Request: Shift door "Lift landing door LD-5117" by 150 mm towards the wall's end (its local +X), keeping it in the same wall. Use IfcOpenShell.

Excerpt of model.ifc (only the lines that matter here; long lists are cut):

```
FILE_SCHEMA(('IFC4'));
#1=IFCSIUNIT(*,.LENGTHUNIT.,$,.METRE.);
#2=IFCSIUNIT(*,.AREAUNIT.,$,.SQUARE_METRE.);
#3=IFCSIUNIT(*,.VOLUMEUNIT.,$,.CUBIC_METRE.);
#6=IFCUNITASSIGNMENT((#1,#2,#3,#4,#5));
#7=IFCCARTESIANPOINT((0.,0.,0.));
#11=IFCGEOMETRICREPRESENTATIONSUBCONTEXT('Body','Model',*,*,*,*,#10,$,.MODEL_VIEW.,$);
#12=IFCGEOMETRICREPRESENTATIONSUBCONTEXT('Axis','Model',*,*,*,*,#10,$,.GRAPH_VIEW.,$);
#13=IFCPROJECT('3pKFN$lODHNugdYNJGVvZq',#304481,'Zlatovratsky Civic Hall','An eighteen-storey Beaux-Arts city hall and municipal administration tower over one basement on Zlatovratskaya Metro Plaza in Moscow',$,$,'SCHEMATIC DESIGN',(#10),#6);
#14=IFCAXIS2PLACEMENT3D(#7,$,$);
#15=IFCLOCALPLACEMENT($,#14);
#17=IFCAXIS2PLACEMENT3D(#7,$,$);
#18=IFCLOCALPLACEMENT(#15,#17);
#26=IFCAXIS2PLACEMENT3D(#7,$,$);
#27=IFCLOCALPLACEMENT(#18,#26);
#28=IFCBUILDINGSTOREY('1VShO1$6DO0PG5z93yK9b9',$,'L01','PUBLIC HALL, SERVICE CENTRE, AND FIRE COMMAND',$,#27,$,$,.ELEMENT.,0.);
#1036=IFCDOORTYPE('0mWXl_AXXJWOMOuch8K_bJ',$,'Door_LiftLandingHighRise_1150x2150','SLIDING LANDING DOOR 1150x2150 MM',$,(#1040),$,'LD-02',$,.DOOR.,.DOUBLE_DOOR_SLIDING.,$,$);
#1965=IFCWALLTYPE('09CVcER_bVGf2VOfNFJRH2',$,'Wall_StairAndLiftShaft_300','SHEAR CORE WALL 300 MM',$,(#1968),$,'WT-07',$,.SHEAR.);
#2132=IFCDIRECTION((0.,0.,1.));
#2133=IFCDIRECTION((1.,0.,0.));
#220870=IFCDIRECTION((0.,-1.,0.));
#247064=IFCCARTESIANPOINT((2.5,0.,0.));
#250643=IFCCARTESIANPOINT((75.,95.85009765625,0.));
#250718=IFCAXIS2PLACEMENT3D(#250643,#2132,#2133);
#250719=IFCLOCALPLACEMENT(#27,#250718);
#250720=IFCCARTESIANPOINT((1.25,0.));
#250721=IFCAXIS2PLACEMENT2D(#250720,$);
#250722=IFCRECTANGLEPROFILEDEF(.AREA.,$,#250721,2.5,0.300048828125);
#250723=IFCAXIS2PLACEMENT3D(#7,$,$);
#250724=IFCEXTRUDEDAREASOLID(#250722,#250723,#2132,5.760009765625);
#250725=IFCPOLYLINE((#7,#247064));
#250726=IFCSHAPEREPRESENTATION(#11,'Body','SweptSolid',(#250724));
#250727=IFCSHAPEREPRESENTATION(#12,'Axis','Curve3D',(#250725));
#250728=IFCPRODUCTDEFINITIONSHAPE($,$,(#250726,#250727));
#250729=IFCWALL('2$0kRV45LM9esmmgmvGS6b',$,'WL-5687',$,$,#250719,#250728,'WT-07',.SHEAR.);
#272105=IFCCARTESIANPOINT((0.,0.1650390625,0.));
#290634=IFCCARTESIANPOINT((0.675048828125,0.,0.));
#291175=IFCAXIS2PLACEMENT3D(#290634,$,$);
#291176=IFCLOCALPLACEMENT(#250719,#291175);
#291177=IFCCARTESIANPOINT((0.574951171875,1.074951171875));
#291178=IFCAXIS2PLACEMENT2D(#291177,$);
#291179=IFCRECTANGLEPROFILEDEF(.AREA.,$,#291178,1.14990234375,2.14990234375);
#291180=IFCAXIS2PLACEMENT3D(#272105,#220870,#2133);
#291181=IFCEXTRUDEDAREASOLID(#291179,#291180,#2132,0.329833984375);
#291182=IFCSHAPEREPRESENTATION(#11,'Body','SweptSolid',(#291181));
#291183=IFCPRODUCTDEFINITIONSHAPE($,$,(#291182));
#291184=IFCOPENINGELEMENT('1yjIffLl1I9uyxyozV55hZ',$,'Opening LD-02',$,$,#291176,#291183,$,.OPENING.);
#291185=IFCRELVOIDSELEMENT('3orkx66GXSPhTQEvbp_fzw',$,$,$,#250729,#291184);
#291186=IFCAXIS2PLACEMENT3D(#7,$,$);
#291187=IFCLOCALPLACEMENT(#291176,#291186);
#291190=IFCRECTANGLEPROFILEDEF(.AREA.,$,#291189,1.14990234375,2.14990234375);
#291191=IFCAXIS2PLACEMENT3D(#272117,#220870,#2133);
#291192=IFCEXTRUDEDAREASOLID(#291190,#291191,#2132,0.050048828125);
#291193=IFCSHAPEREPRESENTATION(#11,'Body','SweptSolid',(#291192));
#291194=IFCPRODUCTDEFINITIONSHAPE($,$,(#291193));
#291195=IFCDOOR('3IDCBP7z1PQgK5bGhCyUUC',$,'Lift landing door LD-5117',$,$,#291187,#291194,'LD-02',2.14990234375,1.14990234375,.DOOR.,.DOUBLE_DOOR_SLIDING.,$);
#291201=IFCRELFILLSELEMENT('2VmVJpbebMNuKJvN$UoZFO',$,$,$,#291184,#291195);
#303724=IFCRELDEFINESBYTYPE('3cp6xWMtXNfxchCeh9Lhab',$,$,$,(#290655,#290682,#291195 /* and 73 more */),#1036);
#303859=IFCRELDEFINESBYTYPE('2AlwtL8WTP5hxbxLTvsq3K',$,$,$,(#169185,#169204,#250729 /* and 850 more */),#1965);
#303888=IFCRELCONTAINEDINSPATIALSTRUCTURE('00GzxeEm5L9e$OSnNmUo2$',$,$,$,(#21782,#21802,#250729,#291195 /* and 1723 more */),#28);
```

```python
import ifcopenshell
import ifcopenshell.api.geometry
import ifcopenshell.util.placement

model = ifcopenshell.open("model.ifc")

door = model.by_id(291195)
opening = door.FillsVoids[0].RelatingOpeningElement
wall = opening.VoidsElements[0].RelatingBuildingElement

wall_matrix = ifcopenshell.util.placement.get_local_placement(wall.ObjectPlacement)
shift = wall_matrix[:3, 0] * 0.15
before = ifcopenshell.util.placement.get_local_placement(door.ObjectPlacement)[:3, 3].copy()

# The door is placed relative to its opening, so it follows when the opening moves.
matrix = ifcopenshell.util.placement.get_local_placement(opening.ObjectPlacement)
matrix[:3, 3] += shift
ifcopenshell.api.geometry.edit_object_placement(
    model, product=opening, matrix=matrix, is_si=False, should_transform_children=True
)

after = ifcopenshell.util.placement.get_local_placement(door.ObjectPlacement)[:3, 3]
print("door moved by", (after - before).round(3) + 0.0)

model.write("model_rev.ifc")
```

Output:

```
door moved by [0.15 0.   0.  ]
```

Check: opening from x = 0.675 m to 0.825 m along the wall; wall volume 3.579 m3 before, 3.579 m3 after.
